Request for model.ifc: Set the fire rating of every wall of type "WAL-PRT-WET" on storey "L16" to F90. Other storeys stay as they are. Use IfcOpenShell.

First a look at what the model holds.

```python
import ifcopenshell
import ifcopenshell.util.element

model = ifcopenshell.open("model.ifc")
print(model.schema)
storey = next(s for s in model.by_type("IfcBuildingStorey") if s.Name == "L16")
walls = [e for e in ifcopenshell.util.element.get_decomposition(storey) if e.is_a("IfcWall")]
seen = {}
for e in walls:
    element_type = ifcopenshell.util.element.get_type(e)
    key = (element_type.Name if element_type != e and element_type else None, ifcopenshell.util.element.get_pset(e, "Pset_WallCommon", "FireRating"))
    seen[key] = seen.get(key, 0) + 1
for (name, value), count in sorted(seen.items(), key=str):
    print(count, "x", name, "|", value)
```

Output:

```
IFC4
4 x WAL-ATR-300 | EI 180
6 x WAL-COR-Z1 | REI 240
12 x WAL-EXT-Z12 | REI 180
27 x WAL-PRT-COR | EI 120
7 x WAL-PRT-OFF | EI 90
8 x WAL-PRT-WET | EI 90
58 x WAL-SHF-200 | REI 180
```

```python
import ifcopenshell
import ifcopenshell.api.pset
import ifcopenshell.util.element

model = ifcopenshell.open("model.ifc")

storey = next(s for s in model.by_type("IfcBuildingStorey") if s.Name == "L16")
walls = [e for e in ifcopenshell.util.element.get_decomposition(storey) if e.is_a("IfcWall")]

count = 0
for e in walls:
    element_type = ifcopenshell.util.element.get_type(e)
    if element_type in (None, e) or element_type.Name != "WAL-PRT-WET":
        continue
    found = ifcopenshell.util.element.get_pset(e, "Pset_WallCommon", should_inherit=False)
    if found:
        pset = model.by_id(found["id"])
        if len(ifcopenshell.util.element.get_elements_by_pset(pset)) > 1:
            pset = ifcopenshell.api.pset.unshare_pset(model, products=[e], pset=pset)[0]
    else:
        pset = ifcopenshell.api.pset.add_pset(model, product=e, name="Pset_WallCommon")
    ifcopenshell.api.pset.edit_pset(model, pset=pset, properties={"FireRating": "F90"})
    count += 1

print(count, "walls updated")

model.write("model_updated.ifc")
```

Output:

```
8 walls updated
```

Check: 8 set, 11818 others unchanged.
